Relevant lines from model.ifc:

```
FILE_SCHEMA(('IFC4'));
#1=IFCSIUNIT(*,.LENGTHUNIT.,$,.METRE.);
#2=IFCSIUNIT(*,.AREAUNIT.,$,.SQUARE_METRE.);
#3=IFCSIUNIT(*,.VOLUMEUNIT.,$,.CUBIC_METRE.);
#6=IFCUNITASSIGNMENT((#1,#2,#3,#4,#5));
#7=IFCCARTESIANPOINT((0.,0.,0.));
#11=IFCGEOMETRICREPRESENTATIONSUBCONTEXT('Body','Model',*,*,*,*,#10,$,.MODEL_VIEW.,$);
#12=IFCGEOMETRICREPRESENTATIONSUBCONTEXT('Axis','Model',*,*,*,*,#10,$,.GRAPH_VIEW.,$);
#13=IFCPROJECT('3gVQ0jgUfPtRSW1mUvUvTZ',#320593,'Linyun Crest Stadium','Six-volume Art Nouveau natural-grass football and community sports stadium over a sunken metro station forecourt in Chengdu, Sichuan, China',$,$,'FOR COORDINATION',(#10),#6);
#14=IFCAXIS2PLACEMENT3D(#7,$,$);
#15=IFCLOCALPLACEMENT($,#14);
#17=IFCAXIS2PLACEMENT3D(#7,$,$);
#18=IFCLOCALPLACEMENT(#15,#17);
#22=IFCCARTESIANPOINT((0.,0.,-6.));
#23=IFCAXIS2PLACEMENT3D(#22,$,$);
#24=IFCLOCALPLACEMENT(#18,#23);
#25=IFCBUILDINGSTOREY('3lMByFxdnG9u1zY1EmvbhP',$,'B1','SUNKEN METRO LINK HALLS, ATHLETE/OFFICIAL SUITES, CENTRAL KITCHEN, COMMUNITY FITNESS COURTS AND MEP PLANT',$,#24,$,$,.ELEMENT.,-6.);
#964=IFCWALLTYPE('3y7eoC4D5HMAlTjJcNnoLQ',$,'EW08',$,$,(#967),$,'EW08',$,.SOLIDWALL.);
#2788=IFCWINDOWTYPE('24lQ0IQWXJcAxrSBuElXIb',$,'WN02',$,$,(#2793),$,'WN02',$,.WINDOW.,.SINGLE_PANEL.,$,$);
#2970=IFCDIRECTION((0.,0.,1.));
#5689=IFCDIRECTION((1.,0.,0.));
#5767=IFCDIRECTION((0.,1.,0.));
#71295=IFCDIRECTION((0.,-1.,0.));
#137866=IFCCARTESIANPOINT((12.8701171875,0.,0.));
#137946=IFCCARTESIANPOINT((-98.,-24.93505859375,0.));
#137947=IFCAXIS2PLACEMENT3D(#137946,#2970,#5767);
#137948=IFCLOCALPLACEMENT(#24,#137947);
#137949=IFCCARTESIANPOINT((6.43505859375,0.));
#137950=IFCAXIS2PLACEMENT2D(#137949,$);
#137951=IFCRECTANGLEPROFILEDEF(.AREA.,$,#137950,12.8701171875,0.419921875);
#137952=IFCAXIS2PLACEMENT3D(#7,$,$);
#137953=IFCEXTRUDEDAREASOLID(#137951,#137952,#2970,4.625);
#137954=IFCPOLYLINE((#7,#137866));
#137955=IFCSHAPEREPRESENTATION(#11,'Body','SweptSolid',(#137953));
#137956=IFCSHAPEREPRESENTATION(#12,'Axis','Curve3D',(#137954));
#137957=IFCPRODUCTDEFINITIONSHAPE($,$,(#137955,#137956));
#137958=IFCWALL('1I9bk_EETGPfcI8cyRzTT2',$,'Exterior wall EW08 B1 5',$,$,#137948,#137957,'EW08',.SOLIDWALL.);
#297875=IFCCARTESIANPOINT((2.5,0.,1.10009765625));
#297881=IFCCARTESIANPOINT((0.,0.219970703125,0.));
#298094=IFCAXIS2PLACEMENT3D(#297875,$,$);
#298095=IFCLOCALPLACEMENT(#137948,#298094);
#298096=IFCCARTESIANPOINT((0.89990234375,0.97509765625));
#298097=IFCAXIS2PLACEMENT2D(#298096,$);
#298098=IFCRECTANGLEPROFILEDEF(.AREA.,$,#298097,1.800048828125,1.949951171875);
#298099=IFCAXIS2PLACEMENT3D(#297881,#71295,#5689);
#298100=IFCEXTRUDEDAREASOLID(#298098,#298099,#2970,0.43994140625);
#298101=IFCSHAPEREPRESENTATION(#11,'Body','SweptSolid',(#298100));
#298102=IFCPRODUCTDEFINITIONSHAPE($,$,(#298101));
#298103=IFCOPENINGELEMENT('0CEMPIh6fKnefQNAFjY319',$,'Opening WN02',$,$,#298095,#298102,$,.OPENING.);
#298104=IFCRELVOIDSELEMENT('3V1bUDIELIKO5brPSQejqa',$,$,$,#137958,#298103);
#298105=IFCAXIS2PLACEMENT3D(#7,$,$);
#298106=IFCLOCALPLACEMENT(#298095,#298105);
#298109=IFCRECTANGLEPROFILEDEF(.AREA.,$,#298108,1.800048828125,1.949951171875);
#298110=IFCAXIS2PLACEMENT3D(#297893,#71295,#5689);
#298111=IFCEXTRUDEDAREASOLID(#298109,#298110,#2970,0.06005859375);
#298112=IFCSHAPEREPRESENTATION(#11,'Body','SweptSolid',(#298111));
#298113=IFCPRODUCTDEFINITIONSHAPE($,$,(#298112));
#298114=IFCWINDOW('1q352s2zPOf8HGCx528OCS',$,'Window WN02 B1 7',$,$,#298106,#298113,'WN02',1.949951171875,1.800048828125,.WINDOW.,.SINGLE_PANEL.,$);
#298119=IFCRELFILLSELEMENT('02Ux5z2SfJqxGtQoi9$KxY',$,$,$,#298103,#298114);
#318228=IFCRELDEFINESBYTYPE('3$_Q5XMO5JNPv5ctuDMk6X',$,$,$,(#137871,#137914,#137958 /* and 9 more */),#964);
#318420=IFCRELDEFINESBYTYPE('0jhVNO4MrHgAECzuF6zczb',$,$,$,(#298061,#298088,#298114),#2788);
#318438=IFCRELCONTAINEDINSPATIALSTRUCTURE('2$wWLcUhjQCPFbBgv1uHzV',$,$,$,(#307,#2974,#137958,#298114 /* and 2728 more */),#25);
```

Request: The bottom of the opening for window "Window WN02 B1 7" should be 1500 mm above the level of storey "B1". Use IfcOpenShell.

```python
import numpy as np
import ifcopenshell
import ifcopenshell.api.geometry
import ifcopenshell.geom
import ifcopenshell.util.element
import ifcopenshell.util.placement
import ifcopenshell.util.shape
import ifcopenshell.util.unit

model = ifcopenshell.open("model.ifc")
unit_scale = ifcopenshell.util.unit.calculate_unit_scale(model)

window = model.by_guid("1q352s2zPOf8HGCx528OCS")
opening = window.FillsVoids[0].RelatingOpeningElement
storey = ifcopenshell.util.element.get_container(window, ifc_class="IfcBuildingStorey")
level = ifcopenshell.util.placement.get_local_placement(storey.ObjectPlacement)[2, 3]

# The opening's origin need not be at the sill, so measure its lowest point.
shape = ifcopenshell.geom.create_shape(ifcopenshell.geom.settings(), opening)
bottom = ifcopenshell.util.shape.get_shape_bottom_elevation(shape, shape.geometry) / unit_scale
dz = level + 1.5 / unit_scale - bottom

shift = np.array([0.0, 0.0, dz])
# The window is placed relative to its opening, so it follows when the opening moves.
matrix = ifcopenshell.util.placement.get_local_placement(opening.ObjectPlacement)
matrix[:3, 3] += shift
ifcopenshell.api.geometry.edit_object_placement(
    model, product=opening, matrix=matrix, is_si=False, should_transform_children=True
)

print(f"moved by {dz * unit_scale:+.3f} m")

model.write("model_updated.ifc")
```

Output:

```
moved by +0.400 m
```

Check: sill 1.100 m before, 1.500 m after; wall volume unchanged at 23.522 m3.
